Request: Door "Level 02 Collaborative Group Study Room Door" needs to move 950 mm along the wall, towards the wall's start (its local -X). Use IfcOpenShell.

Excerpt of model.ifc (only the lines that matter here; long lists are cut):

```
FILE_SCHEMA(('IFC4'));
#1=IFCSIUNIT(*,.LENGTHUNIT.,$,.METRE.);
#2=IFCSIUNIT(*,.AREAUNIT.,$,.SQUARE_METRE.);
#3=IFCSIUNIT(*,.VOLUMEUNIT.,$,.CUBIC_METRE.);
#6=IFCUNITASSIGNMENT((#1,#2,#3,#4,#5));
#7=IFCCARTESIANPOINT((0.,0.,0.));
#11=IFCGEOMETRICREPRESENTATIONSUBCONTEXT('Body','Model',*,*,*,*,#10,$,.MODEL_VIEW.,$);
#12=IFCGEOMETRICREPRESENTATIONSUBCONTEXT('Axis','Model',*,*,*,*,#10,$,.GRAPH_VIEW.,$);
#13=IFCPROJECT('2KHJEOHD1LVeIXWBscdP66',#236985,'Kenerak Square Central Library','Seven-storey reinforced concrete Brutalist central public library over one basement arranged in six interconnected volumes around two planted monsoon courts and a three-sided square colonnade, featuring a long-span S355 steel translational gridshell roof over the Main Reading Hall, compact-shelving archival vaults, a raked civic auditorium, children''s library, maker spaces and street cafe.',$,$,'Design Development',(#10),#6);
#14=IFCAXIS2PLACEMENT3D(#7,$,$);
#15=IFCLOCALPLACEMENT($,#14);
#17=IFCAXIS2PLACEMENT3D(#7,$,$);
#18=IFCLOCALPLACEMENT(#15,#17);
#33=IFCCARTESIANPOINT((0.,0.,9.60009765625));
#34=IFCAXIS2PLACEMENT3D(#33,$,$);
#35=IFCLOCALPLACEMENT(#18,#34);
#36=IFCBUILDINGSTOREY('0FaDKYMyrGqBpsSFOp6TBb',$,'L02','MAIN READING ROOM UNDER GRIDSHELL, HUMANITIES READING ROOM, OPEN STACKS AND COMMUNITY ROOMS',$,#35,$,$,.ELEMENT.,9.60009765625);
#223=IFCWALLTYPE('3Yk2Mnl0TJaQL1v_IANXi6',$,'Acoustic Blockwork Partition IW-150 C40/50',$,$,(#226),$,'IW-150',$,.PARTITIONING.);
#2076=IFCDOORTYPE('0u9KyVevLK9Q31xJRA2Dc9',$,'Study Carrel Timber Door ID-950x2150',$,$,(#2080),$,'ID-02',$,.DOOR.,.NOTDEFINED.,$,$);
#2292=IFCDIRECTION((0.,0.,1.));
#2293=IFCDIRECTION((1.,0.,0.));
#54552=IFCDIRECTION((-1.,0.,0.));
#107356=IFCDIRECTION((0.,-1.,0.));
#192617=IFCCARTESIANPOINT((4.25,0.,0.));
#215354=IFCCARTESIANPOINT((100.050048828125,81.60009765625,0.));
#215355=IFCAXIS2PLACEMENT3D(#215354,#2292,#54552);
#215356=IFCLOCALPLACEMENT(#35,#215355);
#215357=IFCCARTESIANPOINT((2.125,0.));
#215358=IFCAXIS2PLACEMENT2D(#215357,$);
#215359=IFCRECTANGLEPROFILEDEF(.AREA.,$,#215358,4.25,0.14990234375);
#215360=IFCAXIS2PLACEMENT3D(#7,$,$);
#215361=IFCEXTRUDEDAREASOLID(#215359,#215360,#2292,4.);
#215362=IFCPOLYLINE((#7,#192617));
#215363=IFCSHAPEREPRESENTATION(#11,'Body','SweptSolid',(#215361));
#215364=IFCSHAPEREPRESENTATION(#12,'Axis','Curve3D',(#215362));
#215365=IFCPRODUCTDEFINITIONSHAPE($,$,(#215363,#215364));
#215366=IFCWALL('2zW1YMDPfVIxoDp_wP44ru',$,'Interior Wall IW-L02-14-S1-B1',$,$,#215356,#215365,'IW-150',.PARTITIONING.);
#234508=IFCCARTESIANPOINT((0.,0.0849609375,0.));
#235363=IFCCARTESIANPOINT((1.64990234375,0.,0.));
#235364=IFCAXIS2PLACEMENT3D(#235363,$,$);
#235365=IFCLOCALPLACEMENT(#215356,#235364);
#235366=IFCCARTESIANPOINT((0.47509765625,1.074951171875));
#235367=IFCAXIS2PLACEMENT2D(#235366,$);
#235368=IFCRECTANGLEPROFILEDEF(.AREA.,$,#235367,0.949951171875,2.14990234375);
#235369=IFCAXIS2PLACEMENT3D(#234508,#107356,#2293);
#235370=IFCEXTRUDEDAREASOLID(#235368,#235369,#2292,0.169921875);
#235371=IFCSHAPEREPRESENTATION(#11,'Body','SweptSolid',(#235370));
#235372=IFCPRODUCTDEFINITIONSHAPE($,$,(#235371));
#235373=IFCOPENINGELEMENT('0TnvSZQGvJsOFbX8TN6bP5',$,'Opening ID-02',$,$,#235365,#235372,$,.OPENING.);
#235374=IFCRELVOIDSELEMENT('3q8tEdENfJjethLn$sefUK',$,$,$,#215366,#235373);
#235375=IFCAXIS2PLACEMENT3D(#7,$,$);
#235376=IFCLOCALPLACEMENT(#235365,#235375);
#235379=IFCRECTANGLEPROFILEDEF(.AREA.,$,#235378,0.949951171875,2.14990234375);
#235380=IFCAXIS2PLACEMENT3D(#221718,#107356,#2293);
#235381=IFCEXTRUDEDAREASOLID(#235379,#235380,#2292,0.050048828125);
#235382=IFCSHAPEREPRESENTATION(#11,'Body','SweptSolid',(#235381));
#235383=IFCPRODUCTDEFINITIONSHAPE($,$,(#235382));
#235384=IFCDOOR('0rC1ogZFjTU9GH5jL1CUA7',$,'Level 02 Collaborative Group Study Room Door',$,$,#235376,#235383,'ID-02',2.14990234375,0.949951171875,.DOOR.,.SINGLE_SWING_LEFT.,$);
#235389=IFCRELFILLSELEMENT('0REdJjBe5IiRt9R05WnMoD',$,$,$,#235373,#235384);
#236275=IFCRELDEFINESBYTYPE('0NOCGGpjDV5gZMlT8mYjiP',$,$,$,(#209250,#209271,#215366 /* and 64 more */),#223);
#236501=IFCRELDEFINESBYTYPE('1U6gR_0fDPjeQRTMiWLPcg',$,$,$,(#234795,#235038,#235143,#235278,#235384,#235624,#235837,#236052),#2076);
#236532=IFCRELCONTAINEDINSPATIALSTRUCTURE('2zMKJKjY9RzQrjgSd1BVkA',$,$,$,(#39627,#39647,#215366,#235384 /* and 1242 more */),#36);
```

```python
import ifcopenshell
import ifcopenshell.api.geometry
import ifcopenshell.util.placement

model = ifcopenshell.open("model.ifc")

door = model.by_guid("0rC1ogZFjTU9GH5jL1CUA7")
opening = door.FillsVoids[0].RelatingOpeningElement
wall = opening.VoidsElements[0].RelatingBuildingElement

wall_matrix = ifcopenshell.util.placement.get_local_placement(wall.ObjectPlacement)
shift = wall_matrix[:3, 0] * -0.95
before = ifcopenshell.util.placement.get_local_placement(door.ObjectPlacement)[:3, 3].copy()

# The door is placed relative to its opening, so it follows when the opening moves.
matrix = ifcopenshell.util.placement.get_local_placement(opening.ObjectPlacement)
matrix[:3, 3] += shift
ifcopenshell.api.geometry.edit_object_placement(
    model, product=opening, matrix=matrix, is_si=False, should_transform_children=True
)

after = ifcopenshell.util.placement.get_local_placement(door.ObjectPlacement)[:3, 3]
print("door moved by", (after - before).round(3) + 0.0)

model.write("model_updated.ifc")
```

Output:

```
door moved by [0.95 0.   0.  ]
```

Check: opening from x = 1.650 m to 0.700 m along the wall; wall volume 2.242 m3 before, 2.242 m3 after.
